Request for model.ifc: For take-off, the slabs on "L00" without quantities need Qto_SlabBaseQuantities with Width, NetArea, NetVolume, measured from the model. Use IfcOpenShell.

First a look at what the model holds.

```python
import ifcopenshell
import ifcopenshell.util.element
import ifcopenshell.util.unit

model = ifcopenshell.open("model.ifc")
print(model.schema)
for unit_type in ("LENGTHUNIT", "AREAUNIT", "VOLUMEUNIT"):
    print(unit_type, ifcopenshell.util.unit.calculate_unit_scale(model, unit_type))
storey = next(s for s in model.by_type("IfcBuildingStorey") if s.Name == "L00")
slabs = [e for e in ifcopenshell.util.element.get_decomposition(storey) if e.is_a("IfcSlab")]
for e in sorted(slabs, key=lambda e: e.id()):
    print(e.id(), e.is_a(), e.Name, list(ifcopenshell.util.element.get_psets(e, qtos_only=True)), sep=" | ")
```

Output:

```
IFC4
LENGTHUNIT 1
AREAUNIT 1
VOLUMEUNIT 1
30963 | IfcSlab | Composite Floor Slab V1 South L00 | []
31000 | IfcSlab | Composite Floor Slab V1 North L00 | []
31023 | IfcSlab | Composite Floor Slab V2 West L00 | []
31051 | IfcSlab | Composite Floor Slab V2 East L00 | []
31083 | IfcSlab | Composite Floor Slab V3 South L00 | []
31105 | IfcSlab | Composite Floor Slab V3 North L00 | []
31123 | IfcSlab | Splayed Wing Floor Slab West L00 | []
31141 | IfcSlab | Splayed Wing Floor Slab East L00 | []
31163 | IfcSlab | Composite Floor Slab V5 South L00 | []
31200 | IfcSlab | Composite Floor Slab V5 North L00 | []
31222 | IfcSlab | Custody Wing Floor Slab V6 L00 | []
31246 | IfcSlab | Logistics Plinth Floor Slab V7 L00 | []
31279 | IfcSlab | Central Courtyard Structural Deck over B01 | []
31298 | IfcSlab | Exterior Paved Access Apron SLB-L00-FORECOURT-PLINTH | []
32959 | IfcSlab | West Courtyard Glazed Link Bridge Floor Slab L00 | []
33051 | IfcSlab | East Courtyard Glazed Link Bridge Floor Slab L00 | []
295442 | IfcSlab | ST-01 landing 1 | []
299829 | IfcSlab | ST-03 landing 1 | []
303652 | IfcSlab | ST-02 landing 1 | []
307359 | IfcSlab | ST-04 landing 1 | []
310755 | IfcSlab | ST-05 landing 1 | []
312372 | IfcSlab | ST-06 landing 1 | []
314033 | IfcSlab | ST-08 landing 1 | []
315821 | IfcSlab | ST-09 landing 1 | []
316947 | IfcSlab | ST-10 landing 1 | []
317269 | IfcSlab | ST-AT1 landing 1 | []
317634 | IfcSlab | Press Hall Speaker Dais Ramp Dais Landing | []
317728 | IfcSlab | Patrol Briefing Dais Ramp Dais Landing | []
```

```python
import ifcopenshell
import ifcopenshell.api.pset
import ifcopenshell.geom
import ifcopenshell.util.element
import ifcopenshell.util.shape
import ifcopenshell.util.unit

model = ifcopenshell.open("model.ifc")
unit_scale = ifcopenshell.util.unit.calculate_unit_scale(model)
area_scale = ifcopenshell.util.unit.calculate_unit_scale(model, "AREAUNIT")
volume_scale = ifcopenshell.util.unit.calculate_unit_scale(model, "VOLUMEUNIT")
settings = ifcopenshell.geom.settings()

storey = next(s for s in model.by_type("IfcBuildingStorey") if s.Name == "L00")
slabs = [e for e in ifcopenshell.util.element.get_decomposition(storey) if e.is_a("IfcSlab")]

for e in sorted(slabs, key=lambda e: e.id()):
    if ifcopenshell.util.element.get_psets(e, qtos_only=True, should_inherit=False):
        continue
    # Geometry comes back in metres, in the element's own axes.
    shape = ifcopenshell.geom.create_shape(settings, e)
    values = {
        "Width": ifcopenshell.util.shape.get_z(shape.geometry) / unit_scale,
        "NetArea": ifcopenshell.util.shape.get_footprint_area(shape.geometry) / area_scale,
        "NetVolume": ifcopenshell.util.shape.get_volume(shape.geometry) / volume_scale,
    }
    qto = ifcopenshell.api.pset.add_qto(model, product=e, name="Qto_SlabBaseQuantities")
    ifcopenshell.api.pset.edit_qto(model, qto=qto, properties=values)
    print(e.id(), {k: round(v, 3) for k, v in values.items()})

model.write("model_updated.ifc")
```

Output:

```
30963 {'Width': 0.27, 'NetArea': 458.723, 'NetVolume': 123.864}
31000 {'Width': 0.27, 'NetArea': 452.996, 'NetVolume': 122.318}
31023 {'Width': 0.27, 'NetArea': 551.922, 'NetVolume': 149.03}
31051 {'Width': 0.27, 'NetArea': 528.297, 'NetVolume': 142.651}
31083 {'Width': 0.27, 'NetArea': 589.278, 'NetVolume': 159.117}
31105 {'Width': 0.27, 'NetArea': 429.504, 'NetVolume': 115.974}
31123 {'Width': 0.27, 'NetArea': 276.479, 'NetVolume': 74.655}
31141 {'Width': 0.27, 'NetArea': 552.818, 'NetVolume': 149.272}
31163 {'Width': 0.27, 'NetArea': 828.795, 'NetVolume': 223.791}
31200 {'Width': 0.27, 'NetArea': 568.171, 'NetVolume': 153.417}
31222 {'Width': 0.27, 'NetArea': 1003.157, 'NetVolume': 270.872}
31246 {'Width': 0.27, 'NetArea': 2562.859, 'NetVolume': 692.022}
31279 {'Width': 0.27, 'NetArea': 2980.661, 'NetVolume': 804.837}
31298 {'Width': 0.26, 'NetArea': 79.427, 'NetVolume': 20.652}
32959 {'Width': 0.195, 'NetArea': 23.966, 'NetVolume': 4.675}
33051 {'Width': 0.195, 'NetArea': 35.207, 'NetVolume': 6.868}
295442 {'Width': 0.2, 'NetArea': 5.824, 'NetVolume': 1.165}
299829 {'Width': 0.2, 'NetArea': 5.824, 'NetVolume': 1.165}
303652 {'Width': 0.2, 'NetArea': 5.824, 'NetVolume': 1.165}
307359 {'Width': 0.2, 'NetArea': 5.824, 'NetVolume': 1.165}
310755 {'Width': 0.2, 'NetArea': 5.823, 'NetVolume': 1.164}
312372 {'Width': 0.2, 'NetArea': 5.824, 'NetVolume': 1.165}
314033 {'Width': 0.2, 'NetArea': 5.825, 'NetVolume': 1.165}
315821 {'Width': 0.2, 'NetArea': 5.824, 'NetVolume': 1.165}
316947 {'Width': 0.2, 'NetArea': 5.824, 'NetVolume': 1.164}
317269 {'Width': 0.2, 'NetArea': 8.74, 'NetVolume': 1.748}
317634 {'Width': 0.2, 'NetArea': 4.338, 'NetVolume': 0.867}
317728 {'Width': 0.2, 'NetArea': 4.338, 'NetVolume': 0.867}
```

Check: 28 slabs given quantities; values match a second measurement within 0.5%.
